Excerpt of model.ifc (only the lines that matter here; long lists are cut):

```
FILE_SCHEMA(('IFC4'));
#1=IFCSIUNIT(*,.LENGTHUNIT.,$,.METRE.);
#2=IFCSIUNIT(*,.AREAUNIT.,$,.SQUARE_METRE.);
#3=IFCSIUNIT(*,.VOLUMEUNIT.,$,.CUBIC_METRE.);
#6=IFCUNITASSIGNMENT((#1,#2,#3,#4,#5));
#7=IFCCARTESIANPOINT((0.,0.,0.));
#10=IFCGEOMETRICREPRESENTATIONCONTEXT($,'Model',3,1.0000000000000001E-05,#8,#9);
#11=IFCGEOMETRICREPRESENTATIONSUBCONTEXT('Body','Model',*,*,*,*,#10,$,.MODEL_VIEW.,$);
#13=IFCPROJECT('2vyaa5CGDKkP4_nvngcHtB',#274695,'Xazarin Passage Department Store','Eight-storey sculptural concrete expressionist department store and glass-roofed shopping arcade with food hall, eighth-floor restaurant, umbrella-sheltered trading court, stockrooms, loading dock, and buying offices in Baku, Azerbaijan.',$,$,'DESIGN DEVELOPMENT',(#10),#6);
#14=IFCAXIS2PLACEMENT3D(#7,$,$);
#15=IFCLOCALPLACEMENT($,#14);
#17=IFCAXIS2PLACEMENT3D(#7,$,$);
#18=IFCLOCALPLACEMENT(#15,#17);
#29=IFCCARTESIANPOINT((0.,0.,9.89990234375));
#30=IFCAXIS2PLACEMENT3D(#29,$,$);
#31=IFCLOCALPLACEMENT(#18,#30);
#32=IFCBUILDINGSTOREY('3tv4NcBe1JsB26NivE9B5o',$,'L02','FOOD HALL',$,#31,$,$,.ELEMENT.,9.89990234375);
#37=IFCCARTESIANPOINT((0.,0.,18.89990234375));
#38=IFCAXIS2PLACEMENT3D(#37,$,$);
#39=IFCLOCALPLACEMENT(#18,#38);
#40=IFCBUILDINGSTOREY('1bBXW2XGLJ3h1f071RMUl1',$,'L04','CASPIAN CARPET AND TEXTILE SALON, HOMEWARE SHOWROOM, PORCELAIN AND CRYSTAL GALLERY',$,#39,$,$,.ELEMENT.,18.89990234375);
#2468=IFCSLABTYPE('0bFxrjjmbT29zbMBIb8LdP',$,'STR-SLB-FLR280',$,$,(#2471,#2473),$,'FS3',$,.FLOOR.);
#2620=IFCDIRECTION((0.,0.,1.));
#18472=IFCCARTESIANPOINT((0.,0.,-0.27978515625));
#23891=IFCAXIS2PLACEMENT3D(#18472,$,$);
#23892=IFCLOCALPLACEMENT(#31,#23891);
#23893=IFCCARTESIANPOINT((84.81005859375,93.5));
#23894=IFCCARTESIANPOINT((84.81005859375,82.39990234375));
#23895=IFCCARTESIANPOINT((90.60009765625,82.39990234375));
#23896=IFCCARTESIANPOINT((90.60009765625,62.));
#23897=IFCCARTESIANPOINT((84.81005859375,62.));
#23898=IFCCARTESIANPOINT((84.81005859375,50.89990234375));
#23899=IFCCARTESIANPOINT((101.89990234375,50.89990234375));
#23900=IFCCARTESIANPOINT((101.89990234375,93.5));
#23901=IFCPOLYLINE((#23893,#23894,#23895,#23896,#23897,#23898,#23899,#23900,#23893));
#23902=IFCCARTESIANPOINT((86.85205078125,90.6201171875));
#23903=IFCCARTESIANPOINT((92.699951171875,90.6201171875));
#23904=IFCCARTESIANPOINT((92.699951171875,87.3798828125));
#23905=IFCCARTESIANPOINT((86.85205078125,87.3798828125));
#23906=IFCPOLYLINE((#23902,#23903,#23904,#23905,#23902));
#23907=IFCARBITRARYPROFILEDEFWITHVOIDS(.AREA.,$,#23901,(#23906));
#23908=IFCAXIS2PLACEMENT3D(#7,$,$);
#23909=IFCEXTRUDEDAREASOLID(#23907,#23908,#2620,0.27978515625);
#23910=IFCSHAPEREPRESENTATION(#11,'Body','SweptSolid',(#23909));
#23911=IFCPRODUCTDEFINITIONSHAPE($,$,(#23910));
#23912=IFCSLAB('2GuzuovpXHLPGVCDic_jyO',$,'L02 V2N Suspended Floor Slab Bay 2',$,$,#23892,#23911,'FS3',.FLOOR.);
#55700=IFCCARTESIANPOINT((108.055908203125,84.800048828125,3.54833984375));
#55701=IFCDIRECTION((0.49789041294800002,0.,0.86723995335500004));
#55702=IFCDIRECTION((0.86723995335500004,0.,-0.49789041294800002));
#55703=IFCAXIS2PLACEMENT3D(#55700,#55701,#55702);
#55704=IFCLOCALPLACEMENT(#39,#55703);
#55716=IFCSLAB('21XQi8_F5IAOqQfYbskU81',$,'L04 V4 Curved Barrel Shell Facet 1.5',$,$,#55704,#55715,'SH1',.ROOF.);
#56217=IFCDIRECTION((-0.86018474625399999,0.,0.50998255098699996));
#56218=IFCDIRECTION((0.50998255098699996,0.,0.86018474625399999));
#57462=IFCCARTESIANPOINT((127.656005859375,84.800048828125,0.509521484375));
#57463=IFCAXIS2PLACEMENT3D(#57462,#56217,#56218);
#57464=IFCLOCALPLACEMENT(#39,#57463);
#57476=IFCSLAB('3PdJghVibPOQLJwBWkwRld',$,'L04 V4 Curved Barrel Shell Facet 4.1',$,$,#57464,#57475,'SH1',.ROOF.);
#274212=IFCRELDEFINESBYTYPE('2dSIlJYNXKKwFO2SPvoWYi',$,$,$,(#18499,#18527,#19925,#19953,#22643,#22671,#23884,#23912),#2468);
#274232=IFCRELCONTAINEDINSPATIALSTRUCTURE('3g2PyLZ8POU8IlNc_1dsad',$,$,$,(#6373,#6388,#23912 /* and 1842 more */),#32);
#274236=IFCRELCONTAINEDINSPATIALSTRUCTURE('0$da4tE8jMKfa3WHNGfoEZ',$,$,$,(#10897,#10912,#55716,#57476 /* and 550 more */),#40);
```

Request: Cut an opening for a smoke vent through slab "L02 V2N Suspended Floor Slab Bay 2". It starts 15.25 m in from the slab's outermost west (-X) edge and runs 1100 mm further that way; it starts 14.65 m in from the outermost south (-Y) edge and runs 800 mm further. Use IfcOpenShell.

```python
import numpy as np
import ifcopenshell
import ifcopenshell.api.feature
import ifcopenshell.api.geometry
import ifcopenshell.api.root
import ifcopenshell.geom
import ifcopenshell.util.placement
import ifcopenshell.util.representation
import ifcopenshell.util.shape
import ifcopenshell.util.unit

model = ifcopenshell.open("model.ifc")
unit_scale = ifcopenshell.util.unit.calculate_unit_scale(model)
settings = ifcopenshell.geom.settings()


def volume(element):
    """Net volume in cubic metres, openings subtracted."""
    shape = ifcopenshell.geom.create_shape(settings, element)
    return ifcopenshell.util.shape.get_volume(shape.geometry)


slab = model.by_guid("2GuzuovpXHLPGVCDic_jyO")
before = volume(slab)

# Extent in the slab's own axes, in metres. The edges named are its -X and -Y sides.
slab_shape = ifcopenshell.geom.create_shape(settings, slab)
vertices = ifcopenshell.util.shape.get_vertices(slab_shape.geometry)
x_min, y_min, bottom = vertices.min(axis=0)
top = vertices[:, 2].max()

opening = ifcopenshell.api.root.create_entity(model, ifc_class="IfcOpeningElement", name="Smoke vent opening", predefined_type="OPENING")
context = ifcopenshell.util.representation.get_context(model, "Model", "Body", "MODEL_VIEW")
width, depth = 1.1, 0.8
outline = [(0.0, 0.0), (width, 0.0), (width, depth), (0.0, depth), (0.0, 0.0)]
# Overshoot both faces by 50 mm so the cut is clean.
shape = ifcopenshell.api.geometry.add_slab_representation(
    model, context=context, depth=top - bottom + 0.1, polyline=outline
)
ifcopenshell.api.geometry.assign_representation(model, product=opening, representation=shape)

matrix = ifcopenshell.util.placement.get_local_placement(slab.ObjectPlacement)
matrix[:, 3] = matrix @ np.append(np.array([x_min + 15.25, y_min + 14.65, bottom - 0.05]) / unit_scale, 1.0)
ifcopenshell.api.geometry.edit_object_placement(model, product=opening, matrix=matrix, is_si=False)
ifcopenshell.api.feature.add_feature(model, feature=opening, element=slab)

after = volume(slab)

print(f"slab volume {before:.3f} -> {after:.3f} m3")

model.write("model-out.ifc")
```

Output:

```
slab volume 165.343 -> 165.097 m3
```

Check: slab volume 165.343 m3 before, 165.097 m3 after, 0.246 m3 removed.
